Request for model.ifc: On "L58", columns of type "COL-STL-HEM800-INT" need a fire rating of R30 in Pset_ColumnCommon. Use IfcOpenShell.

First a look at what the model holds.

```python
import ifcopenshell
import ifcopenshell.util.element

model = ifcopenshell.open("model.ifc")
print(model.schema)
storey = next(s for s in model.by_type("IfcBuildingStorey") if s.Name == "L58")
columns = [e for e in ifcopenshell.util.element.get_decomposition(storey) if e.is_a("IfcColumn")]
seen = {}
for e in columns:
    element_type = ifcopenshell.util.element.get_type(e)
    key = (element_type.Name if element_type != e and element_type else None, ifcopenshell.util.element.get_pset(e, "Pset_ColumnCommon", "FireRating"))
    seen[key] = seen.get(key, 0) + 1
for (name, value), count in sorted(seen.items(), key=str):
    print(count, "x", name, "|", value)
```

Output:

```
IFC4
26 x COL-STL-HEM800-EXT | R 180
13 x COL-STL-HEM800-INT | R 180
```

```python
import ifcopenshell
import ifcopenshell.api.pset
import ifcopenshell.util.element

model = ifcopenshell.open("model.ifc")

storey = next(s for s in model.by_type("IfcBuildingStorey") if s.Name == "L58")
columns = [e for e in ifcopenshell.util.element.get_decomposition(storey) if e.is_a("IfcColumn")]

count = 0
for e in columns:
    element_type = ifcopenshell.util.element.get_type(e)
    if element_type in (None, e) or element_type.Name != "COL-STL-HEM800-INT":
        continue
    # add_pset returns the element's existing set when there is one.
    pset = ifcopenshell.api.pset.add_pset(model, product=e, name="Pset_ColumnCommon")
    ifcopenshell.api.pset.edit_pset(model, pset=pset, properties={"FireRating": "R30"})
    count += 1

print(count, "columns updated")

model.write("model_updated.ifc")
```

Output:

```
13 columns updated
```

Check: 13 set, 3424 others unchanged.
